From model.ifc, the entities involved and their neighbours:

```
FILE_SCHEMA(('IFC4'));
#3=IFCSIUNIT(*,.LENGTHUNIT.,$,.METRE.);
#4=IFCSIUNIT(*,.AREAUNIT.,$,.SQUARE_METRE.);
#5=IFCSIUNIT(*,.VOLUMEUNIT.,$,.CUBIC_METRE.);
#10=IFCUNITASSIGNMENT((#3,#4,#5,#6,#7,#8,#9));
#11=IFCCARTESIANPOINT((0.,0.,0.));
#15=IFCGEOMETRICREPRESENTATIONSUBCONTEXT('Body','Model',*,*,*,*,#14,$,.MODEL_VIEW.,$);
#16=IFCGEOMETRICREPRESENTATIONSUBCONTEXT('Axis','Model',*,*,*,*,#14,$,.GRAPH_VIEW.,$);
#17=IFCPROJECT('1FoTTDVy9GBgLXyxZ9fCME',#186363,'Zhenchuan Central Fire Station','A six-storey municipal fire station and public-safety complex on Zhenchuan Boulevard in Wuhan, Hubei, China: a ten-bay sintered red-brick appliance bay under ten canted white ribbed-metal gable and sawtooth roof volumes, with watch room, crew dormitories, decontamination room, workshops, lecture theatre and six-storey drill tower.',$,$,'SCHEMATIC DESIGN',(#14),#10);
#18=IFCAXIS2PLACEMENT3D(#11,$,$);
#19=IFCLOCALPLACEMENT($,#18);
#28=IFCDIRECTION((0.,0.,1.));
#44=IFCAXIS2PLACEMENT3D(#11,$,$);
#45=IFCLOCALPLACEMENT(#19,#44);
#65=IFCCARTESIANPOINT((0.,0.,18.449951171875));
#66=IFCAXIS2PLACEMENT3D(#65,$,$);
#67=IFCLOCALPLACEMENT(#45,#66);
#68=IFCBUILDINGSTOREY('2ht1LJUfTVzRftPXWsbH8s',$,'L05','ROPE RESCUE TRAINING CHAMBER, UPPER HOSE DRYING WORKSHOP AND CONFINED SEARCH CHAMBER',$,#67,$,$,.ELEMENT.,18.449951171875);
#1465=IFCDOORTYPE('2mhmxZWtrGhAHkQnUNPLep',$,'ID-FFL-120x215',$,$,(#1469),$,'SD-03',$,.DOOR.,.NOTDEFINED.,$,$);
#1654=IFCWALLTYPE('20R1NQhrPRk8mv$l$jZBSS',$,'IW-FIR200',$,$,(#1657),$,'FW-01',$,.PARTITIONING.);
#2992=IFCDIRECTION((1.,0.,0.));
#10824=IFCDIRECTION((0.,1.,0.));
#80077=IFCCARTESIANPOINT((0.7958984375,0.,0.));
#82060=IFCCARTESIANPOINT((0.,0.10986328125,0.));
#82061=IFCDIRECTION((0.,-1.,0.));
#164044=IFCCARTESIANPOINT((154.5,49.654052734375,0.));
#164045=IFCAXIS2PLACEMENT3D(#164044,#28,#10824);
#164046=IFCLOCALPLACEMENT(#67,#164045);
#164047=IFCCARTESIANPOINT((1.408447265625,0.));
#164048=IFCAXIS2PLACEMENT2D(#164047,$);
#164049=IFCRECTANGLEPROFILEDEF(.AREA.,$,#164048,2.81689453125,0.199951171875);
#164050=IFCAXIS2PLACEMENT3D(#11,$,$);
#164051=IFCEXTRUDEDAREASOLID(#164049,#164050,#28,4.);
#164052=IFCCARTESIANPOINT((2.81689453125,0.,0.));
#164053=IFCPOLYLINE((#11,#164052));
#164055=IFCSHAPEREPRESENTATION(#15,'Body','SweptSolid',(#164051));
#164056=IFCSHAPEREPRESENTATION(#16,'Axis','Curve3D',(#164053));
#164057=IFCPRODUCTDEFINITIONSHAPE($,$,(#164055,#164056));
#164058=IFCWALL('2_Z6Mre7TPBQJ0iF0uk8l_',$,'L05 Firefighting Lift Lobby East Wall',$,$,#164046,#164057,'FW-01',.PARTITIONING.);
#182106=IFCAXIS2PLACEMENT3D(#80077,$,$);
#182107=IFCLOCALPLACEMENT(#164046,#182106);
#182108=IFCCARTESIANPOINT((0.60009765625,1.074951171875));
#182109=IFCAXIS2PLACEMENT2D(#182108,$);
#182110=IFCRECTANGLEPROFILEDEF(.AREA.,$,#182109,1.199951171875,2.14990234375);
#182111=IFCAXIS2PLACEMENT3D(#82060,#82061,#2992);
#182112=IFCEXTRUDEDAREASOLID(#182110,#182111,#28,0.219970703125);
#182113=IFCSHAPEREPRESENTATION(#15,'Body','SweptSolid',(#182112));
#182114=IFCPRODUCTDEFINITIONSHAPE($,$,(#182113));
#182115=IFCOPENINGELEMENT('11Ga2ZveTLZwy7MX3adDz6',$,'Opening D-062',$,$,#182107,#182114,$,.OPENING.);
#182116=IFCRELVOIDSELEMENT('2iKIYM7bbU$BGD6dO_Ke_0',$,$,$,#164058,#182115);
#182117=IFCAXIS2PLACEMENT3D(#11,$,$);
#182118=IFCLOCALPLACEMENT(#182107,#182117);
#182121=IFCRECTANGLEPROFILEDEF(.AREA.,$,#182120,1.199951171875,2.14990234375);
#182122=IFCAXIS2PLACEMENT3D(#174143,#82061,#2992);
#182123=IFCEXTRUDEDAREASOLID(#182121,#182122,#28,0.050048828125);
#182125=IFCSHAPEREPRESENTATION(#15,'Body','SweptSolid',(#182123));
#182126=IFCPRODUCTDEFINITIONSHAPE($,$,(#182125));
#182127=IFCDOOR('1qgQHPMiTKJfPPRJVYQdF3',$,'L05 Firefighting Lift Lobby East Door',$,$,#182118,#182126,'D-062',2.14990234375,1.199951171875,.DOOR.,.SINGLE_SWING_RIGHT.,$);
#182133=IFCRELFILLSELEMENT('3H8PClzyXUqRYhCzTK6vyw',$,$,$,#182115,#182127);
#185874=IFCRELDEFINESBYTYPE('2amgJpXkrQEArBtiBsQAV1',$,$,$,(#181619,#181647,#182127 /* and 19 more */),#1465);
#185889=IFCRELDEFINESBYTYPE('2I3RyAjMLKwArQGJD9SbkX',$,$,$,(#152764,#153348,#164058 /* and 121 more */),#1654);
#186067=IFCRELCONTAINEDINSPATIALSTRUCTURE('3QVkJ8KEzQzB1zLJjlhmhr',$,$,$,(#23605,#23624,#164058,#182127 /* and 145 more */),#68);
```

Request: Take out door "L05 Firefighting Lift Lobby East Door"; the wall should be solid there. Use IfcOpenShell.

```python
import ifcopenshell
import ifcopenshell.api.feature
import ifcopenshell.api.root
import ifcopenshell.geom
import ifcopenshell.util.shape

model = ifcopenshell.open("model.ifc")
settings = ifcopenshell.geom.settings()


def volume(element):
    """Net volume in cubic metres, openings subtracted."""
    shape = ifcopenshell.geom.create_shape(settings, element)
    return ifcopenshell.util.shape.get_volume(shape.geometry)


door = model.by_guid("1qgQHPMiTKJfPPRJVYQdF3")
opening = door.FillsVoids[0].RelatingOpeningElement
wall = opening.VoidsElements[0].RelatingBuildingElement
before = volume(wall)

ifcopenshell.api.root.remove_product(model, product=door)
ifcopenshell.api.feature.remove_feature(model, feature=opening)

after = volume(wall)

print(f"wall volume {before:.3f} -> {after:.3f} m3")

model.write("model_updated.ifc")
```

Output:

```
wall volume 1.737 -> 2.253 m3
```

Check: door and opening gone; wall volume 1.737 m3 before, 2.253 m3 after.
